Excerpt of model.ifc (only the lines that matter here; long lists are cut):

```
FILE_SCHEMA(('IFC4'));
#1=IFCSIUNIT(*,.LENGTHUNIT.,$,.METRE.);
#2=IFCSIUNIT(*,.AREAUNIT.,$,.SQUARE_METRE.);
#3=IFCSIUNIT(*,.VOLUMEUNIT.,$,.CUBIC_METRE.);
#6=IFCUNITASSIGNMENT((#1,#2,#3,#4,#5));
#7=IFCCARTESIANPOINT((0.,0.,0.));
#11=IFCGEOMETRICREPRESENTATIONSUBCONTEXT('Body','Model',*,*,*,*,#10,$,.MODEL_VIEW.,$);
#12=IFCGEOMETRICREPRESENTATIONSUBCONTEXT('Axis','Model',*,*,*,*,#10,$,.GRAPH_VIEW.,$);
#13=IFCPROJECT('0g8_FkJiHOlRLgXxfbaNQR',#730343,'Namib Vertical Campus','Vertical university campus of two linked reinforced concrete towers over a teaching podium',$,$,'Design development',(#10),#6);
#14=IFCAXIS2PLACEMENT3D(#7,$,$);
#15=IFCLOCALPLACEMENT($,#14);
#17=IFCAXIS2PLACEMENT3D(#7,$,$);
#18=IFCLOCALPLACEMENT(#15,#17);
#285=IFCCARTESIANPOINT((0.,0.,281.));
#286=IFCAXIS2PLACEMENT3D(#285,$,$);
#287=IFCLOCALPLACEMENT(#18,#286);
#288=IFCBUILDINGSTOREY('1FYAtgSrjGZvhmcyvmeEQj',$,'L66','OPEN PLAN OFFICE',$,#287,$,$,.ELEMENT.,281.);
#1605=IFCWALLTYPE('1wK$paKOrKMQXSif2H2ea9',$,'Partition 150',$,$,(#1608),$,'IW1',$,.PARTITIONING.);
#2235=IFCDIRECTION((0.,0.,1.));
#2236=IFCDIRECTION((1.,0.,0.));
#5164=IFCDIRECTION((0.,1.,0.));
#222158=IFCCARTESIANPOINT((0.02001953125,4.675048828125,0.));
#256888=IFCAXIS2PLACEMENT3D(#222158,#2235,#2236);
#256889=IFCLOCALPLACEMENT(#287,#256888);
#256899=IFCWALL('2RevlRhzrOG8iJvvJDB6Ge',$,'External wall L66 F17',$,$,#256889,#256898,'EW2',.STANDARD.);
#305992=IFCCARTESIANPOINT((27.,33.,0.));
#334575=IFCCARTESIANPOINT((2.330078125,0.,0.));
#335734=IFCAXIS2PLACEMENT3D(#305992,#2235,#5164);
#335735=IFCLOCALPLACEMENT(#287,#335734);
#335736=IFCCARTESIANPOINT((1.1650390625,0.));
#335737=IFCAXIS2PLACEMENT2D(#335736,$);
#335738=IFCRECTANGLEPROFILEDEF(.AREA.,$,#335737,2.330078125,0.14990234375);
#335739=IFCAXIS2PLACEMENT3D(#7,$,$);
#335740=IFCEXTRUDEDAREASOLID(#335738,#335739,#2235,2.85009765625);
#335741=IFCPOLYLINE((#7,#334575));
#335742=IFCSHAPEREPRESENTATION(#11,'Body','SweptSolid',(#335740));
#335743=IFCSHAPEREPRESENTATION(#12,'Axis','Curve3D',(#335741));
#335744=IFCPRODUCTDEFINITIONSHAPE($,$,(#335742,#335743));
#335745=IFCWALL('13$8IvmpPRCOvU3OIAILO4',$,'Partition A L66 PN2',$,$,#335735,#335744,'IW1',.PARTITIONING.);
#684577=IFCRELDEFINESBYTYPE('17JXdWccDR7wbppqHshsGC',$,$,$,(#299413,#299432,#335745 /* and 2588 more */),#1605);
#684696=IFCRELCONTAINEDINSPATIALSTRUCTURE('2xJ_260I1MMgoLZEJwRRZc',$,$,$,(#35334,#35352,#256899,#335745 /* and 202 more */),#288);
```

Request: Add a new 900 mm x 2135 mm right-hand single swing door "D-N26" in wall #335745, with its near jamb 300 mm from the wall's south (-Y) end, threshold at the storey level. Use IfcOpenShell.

```python
import numpy as np
import ifcopenshell
import ifcopenshell.api.feature
import ifcopenshell.api.geometry
import ifcopenshell.api.root
import ifcopenshell.api.spatial
import ifcopenshell.geom
import ifcopenshell.util.element
import ifcopenshell.util.placement
import ifcopenshell.util.representation
import ifcopenshell.util.shape
import ifcopenshell.util.unit

model = ifcopenshell.open("model.ifc")
unit_scale = ifcopenshell.util.unit.calculate_unit_scale(model)
settings = ifcopenshell.geom.settings()


def volume(element):
    """Net volume in cubic metres, openings subtracted."""
    shape = ifcopenshell.geom.create_shape(settings, element)
    return ifcopenshell.util.shape.get_volume(shape.geometry)


wall = model.by_guid("13$8IvmpPRCOvU3OIAILO4")
storey = ifcopenshell.util.element.get_container(wall, ifc_class="IfcBuildingStorey")
context = ifcopenshell.util.representation.get_context(model, "Model", "Body", "MODEL_VIEW")
before = volume(wall)

width, height, from_end, sill = 0.9, 2.135, 0.3, 0.0  # metres

# The wall runs along its own X axis, and the end named is its -X end.
wall_shape = ifcopenshell.geom.create_shape(settings, wall)
x, y, z = ifcopenshell.util.shape.get_vertices(wall_shape.geometry).T
start = x.min() + from_end
face, thickness = float(y.min()), float(y.max() - y.min())
wall_matrix = ifcopenshell.util.placement.get_local_placement(wall.ObjectPlacement)
level = ifcopenshell.util.placement.get_local_placement(storey.ObjectPlacement)[2, 3]


def in_wall(x, y):
    """Placement at x, y metres in the wall's axes, at sill height."""
    matrix = wall_matrix.copy()
    matrix[:, 3] = wall_matrix @ np.array([x / unit_scale, y / unit_scale, 0.0, 1.0])
    matrix[2, 3] = level + sill / unit_scale
    return matrix


# Opening: a box that overshoots both wall faces by 50 mm.
opening = ifcopenshell.api.root.create_entity(model, ifc_class="IfcOpeningElement", predefined_type="OPENING")
box = ifcopenshell.api.geometry.add_wall_representation(
    model, context=context, length=width, height=height, thickness=thickness + 0.1
)
ifcopenshell.api.geometry.assign_representation(model, product=opening, representation=box)
ifcopenshell.api.geometry.edit_object_placement(model, product=opening, matrix=in_wall(start, face - 0.05), is_si=False)
ifcopenshell.api.feature.add_feature(model, feature=opening, element=wall)

door = ifcopenshell.api.root.create_entity(model, ifc_class="IfcDoor", name="D-N26", predefined_type="DOOR")
door.OverallWidth, door.OverallHeight = width / unit_scale, height / unit_scale
door.OperationType = "SINGLE_SWING_RIGHT"
body = ifcopenshell.api.geometry.add_door_representation(
    model,
    context=context,
    overall_width=door.OverallWidth,
    overall_height=door.OverallHeight,
    operation_type="SINGLE_SWING_RIGHT",
    lining_properties={"LiningDepth": thickness / unit_scale, "ThresholdDepth": thickness / unit_scale},
)
ifcopenshell.api.geometry.assign_representation(model, product=door, representation=body)
ifcopenshell.api.spatial.assign_container(model, products=[door], relating_structure=storey)
ifcopenshell.api.feature.add_filling(model, opening=opening, element=door)

# The lining spans the wall, so the door starts at the wall face.
ifcopenshell.api.geometry.edit_object_placement(model, product=door, matrix=in_wall(start, face), is_si=False)

after = volume(wall)

print(f"wall volume {before:.3f} -> {after:.3f} m3")

model.write("model_v2.ifc")
```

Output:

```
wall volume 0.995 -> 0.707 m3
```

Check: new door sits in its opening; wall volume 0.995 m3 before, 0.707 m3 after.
